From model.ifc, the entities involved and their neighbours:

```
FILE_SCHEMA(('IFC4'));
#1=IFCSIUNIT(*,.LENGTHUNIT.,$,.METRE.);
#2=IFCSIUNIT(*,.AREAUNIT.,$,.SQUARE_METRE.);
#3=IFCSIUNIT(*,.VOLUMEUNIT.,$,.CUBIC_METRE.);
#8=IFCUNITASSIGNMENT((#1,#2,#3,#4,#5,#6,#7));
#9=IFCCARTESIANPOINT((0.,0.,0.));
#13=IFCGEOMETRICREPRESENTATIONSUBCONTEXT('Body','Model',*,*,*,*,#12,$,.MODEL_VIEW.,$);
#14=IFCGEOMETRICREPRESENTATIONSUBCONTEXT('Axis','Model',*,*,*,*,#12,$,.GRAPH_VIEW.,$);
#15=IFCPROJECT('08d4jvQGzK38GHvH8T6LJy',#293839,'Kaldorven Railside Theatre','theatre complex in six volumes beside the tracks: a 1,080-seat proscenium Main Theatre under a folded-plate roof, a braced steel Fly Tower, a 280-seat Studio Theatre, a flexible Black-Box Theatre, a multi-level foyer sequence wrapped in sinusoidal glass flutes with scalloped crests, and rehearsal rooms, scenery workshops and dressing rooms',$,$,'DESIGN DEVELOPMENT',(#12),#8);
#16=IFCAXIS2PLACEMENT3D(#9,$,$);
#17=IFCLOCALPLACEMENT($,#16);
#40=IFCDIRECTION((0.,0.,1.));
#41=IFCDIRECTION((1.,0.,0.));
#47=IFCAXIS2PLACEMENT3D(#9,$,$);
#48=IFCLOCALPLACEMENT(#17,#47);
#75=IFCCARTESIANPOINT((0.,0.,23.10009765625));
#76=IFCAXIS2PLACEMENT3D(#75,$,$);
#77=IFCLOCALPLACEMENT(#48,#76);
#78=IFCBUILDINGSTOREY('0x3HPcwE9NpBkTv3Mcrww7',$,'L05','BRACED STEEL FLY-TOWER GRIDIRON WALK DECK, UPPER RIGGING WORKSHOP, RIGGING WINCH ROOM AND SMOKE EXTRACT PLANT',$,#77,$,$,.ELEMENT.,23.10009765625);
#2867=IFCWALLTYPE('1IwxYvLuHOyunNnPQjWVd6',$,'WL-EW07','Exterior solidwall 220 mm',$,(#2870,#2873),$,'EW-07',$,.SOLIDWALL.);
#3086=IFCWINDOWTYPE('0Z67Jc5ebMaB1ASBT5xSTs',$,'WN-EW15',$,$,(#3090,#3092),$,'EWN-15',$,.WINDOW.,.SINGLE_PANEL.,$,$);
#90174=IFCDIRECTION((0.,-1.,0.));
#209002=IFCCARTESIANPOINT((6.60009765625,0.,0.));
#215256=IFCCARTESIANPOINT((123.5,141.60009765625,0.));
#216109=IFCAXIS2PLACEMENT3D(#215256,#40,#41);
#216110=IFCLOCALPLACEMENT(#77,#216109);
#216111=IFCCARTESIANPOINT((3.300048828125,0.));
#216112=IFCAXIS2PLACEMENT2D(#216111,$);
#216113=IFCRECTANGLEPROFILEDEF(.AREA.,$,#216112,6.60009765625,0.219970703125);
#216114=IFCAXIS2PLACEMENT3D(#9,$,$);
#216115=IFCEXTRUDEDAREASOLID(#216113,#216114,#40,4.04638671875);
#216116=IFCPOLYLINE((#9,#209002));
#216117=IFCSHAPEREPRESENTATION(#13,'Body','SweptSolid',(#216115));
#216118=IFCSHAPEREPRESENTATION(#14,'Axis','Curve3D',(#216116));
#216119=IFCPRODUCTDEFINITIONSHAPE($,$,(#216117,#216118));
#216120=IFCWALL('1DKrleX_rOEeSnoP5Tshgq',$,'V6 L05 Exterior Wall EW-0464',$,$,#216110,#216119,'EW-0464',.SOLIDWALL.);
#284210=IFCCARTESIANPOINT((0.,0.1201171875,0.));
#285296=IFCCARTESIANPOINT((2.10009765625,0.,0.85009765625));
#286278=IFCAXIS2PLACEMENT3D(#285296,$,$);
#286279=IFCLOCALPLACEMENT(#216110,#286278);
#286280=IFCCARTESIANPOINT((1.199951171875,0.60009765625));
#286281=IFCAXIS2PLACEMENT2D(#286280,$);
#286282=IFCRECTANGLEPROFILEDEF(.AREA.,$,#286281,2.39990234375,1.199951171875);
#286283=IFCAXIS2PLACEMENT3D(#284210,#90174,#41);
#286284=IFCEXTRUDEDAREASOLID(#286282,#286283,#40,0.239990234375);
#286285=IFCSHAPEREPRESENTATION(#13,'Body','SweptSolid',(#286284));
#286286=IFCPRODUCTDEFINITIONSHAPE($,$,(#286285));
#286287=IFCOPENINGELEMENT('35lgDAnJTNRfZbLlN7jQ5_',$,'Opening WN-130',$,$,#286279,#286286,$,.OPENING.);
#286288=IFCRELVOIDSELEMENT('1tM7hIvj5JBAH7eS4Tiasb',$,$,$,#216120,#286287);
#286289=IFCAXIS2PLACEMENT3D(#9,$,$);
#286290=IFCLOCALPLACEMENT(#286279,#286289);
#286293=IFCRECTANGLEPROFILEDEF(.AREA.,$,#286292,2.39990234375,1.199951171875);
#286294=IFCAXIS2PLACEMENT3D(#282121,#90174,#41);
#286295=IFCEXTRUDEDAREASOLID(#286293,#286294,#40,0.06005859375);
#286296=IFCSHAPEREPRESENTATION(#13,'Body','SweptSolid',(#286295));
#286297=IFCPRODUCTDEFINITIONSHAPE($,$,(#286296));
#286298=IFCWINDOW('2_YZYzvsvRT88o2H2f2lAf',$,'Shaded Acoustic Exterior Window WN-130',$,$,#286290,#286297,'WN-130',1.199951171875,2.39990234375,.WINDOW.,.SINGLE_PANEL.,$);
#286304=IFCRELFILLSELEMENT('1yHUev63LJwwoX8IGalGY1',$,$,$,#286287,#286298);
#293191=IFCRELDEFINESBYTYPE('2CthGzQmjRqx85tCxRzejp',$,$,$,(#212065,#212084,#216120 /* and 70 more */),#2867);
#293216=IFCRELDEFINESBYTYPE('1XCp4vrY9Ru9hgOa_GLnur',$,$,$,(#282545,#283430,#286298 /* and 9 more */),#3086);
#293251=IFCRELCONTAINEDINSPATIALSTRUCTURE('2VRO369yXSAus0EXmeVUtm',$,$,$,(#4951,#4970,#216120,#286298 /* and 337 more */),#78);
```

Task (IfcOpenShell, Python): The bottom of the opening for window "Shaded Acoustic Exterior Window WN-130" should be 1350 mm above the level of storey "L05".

```python
import numpy as np
import ifcopenshell
import ifcopenshell.api.geometry
import ifcopenshell.geom
import ifcopenshell.util.element
import ifcopenshell.util.placement
import ifcopenshell.util.shape
import ifcopenshell.util.unit

model = ifcopenshell.open("model.ifc")
unit_scale = ifcopenshell.util.unit.calculate_unit_scale(model)

window = model.by_guid("2_YZYzvsvRT88o2H2f2lAf")
opening = window.FillsVoids[0].RelatingOpeningElement
storey = ifcopenshell.util.element.get_container(window, ifc_class="IfcBuildingStorey")
level = ifcopenshell.util.placement.get_local_placement(storey.ObjectPlacement)[2, 3]

# The opening's origin need not be at the sill, so measure its lowest point.
shape = ifcopenshell.geom.create_shape(ifcopenshell.geom.settings(), opening)
bottom = ifcopenshell.util.shape.get_shape_bottom_elevation(shape, shape.geometry) / unit_scale
dz = level + 1.35 / unit_scale - bottom

shift = np.array([0.0, 0.0, dz])
# The window is placed relative to its opening, so it follows when the opening moves.
matrix = ifcopenshell.util.placement.get_local_placement(opening.ObjectPlacement)
matrix[:3, 3] += shift
ifcopenshell.api.geometry.edit_object_placement(
    model, product=opening, matrix=matrix, is_si=False, should_transform_children=True
)

print(f"moved by {dz * unit_scale:+.3f} m")

model.write("model_updated.ifc")
```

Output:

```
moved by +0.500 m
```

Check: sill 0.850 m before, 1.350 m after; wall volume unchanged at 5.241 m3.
